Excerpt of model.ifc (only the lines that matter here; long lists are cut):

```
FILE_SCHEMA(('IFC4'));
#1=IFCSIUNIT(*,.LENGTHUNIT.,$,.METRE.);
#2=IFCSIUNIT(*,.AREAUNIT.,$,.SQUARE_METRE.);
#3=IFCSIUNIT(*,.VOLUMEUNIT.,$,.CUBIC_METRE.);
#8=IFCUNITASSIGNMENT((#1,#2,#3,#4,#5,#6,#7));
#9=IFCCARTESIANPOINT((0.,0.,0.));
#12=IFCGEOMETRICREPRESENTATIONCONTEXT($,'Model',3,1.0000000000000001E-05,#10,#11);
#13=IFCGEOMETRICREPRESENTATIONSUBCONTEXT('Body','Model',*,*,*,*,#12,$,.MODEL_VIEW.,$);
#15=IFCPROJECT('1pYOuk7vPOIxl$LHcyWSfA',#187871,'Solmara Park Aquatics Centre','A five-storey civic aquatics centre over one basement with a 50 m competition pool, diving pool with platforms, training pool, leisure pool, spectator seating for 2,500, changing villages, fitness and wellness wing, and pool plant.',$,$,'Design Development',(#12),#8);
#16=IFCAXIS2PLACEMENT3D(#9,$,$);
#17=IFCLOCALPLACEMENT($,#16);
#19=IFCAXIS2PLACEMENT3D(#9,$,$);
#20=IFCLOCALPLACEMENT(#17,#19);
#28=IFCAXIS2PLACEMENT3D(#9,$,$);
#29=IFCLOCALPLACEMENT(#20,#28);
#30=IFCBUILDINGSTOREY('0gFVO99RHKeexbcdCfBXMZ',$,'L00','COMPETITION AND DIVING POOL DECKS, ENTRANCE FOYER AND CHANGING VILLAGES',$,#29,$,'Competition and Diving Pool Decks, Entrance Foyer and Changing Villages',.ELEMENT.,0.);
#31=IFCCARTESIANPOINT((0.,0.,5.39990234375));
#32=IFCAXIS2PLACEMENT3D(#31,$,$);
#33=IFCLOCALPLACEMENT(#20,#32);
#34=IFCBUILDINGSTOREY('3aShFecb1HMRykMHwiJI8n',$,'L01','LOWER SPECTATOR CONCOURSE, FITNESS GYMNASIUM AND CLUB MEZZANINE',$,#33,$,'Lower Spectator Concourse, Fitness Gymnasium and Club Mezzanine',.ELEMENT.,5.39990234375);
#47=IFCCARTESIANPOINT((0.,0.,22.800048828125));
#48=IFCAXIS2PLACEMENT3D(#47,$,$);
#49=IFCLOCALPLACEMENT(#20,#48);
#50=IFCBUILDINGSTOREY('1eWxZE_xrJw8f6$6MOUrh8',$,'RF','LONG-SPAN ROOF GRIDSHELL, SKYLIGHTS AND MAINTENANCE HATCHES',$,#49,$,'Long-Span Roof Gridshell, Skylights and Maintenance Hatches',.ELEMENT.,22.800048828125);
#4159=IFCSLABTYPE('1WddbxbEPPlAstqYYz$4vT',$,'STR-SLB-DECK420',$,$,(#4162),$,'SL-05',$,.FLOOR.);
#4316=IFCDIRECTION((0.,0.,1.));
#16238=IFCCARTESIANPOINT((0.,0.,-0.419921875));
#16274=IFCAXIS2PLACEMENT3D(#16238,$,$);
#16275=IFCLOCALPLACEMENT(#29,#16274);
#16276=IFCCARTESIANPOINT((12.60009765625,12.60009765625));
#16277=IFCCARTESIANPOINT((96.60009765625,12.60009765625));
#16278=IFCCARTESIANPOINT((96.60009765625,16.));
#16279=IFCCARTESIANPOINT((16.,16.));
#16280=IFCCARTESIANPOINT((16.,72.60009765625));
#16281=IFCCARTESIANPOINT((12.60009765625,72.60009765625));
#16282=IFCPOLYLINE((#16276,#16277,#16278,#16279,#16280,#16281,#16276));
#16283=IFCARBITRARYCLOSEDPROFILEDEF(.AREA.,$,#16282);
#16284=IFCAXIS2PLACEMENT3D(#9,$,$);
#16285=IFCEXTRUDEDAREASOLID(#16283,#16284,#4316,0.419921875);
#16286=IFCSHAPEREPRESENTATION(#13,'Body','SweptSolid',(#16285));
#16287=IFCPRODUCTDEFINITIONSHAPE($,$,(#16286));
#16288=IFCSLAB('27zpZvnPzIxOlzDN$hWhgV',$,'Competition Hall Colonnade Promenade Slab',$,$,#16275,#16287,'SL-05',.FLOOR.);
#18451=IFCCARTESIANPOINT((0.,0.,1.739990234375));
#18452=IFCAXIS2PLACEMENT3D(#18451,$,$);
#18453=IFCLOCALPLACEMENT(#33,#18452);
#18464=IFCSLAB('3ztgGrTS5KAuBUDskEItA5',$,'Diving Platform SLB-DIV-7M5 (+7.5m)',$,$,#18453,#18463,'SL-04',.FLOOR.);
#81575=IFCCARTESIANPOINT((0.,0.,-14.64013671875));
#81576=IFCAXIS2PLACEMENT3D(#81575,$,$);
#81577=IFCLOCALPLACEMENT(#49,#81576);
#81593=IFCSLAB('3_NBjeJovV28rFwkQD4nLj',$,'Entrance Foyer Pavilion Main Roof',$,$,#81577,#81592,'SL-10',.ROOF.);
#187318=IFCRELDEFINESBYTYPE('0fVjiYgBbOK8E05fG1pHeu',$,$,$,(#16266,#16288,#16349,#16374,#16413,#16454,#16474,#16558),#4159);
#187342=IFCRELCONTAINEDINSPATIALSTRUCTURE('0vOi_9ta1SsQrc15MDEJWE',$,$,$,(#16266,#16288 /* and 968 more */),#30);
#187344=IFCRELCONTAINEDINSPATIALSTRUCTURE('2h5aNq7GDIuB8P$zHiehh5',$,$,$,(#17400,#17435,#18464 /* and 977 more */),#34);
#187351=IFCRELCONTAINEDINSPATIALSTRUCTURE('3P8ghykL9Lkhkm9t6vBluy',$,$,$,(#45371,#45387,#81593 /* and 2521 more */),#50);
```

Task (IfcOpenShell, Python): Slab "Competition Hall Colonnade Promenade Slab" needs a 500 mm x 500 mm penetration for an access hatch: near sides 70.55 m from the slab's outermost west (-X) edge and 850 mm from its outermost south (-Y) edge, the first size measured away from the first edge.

```python
import numpy as np
import ifcopenshell
import ifcopenshell.api.feature
import ifcopenshell.api.geometry
import ifcopenshell.api.root
import ifcopenshell.geom
import ifcopenshell.util.placement
import ifcopenshell.util.representation
import ifcopenshell.util.shape
import ifcopenshell.util.unit

model = ifcopenshell.open("model.ifc")
unit_scale = ifcopenshell.util.unit.calculate_unit_scale(model)
settings = ifcopenshell.geom.settings()


def volume(element):
    """Net volume in cubic metres, openings subtracted."""
    shape = ifcopenshell.geom.create_shape(settings, element)
    return ifcopenshell.util.shape.get_volume(shape.geometry)


slab = model.by_guid("27zpZvnPzIxOlzDN$hWhgV")
before = volume(slab)

# Extent in the slab's own axes, in metres. The edges named are its -X and -Y sides.
slab_shape = ifcopenshell.geom.create_shape(settings, slab)
vertices = ifcopenshell.util.shape.get_vertices(slab_shape.geometry)
x_min, y_min, bottom = vertices.min(axis=0)
top = vertices[:, 2].max()

opening = ifcopenshell.api.root.create_entity(model, ifc_class="IfcOpeningElement", name="Access hatch opening", predefined_type="OPENING")
context = ifcopenshell.util.representation.get_context(model, "Model", "Body", "MODEL_VIEW")
width, depth = 0.5, 0.5
outline = [(0.0, 0.0), (width, 0.0), (width, depth), (0.0, depth), (0.0, 0.0)]
# Overshoot both faces by 50 mm so the cut is clean.
shape = ifcopenshell.api.geometry.add_slab_representation(
    model, context=context, depth=top - bottom + 0.1, polyline=outline
)
ifcopenshell.api.geometry.assign_representation(model, product=opening, representation=shape)

matrix = ifcopenshell.util.placement.get_local_placement(slab.ObjectPlacement)
matrix[:, 3] = matrix @ np.append(np.array([x_min + 70.55, y_min + 0.85, bottom - 0.05]) / unit_scale, 1.0)
ifcopenshell.api.geometry.edit_object_placement(model, product=opening, matrix=matrix, is_si=False)
ifcopenshell.api.feature.add_feature(model, feature=opening, element=slab)

after = volume(slab)

print(f"slab volume {before:.3f} -> {after:.3f} m3")

model.write("model_updated.ifc")
```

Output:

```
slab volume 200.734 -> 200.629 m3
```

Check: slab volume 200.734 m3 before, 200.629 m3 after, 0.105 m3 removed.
